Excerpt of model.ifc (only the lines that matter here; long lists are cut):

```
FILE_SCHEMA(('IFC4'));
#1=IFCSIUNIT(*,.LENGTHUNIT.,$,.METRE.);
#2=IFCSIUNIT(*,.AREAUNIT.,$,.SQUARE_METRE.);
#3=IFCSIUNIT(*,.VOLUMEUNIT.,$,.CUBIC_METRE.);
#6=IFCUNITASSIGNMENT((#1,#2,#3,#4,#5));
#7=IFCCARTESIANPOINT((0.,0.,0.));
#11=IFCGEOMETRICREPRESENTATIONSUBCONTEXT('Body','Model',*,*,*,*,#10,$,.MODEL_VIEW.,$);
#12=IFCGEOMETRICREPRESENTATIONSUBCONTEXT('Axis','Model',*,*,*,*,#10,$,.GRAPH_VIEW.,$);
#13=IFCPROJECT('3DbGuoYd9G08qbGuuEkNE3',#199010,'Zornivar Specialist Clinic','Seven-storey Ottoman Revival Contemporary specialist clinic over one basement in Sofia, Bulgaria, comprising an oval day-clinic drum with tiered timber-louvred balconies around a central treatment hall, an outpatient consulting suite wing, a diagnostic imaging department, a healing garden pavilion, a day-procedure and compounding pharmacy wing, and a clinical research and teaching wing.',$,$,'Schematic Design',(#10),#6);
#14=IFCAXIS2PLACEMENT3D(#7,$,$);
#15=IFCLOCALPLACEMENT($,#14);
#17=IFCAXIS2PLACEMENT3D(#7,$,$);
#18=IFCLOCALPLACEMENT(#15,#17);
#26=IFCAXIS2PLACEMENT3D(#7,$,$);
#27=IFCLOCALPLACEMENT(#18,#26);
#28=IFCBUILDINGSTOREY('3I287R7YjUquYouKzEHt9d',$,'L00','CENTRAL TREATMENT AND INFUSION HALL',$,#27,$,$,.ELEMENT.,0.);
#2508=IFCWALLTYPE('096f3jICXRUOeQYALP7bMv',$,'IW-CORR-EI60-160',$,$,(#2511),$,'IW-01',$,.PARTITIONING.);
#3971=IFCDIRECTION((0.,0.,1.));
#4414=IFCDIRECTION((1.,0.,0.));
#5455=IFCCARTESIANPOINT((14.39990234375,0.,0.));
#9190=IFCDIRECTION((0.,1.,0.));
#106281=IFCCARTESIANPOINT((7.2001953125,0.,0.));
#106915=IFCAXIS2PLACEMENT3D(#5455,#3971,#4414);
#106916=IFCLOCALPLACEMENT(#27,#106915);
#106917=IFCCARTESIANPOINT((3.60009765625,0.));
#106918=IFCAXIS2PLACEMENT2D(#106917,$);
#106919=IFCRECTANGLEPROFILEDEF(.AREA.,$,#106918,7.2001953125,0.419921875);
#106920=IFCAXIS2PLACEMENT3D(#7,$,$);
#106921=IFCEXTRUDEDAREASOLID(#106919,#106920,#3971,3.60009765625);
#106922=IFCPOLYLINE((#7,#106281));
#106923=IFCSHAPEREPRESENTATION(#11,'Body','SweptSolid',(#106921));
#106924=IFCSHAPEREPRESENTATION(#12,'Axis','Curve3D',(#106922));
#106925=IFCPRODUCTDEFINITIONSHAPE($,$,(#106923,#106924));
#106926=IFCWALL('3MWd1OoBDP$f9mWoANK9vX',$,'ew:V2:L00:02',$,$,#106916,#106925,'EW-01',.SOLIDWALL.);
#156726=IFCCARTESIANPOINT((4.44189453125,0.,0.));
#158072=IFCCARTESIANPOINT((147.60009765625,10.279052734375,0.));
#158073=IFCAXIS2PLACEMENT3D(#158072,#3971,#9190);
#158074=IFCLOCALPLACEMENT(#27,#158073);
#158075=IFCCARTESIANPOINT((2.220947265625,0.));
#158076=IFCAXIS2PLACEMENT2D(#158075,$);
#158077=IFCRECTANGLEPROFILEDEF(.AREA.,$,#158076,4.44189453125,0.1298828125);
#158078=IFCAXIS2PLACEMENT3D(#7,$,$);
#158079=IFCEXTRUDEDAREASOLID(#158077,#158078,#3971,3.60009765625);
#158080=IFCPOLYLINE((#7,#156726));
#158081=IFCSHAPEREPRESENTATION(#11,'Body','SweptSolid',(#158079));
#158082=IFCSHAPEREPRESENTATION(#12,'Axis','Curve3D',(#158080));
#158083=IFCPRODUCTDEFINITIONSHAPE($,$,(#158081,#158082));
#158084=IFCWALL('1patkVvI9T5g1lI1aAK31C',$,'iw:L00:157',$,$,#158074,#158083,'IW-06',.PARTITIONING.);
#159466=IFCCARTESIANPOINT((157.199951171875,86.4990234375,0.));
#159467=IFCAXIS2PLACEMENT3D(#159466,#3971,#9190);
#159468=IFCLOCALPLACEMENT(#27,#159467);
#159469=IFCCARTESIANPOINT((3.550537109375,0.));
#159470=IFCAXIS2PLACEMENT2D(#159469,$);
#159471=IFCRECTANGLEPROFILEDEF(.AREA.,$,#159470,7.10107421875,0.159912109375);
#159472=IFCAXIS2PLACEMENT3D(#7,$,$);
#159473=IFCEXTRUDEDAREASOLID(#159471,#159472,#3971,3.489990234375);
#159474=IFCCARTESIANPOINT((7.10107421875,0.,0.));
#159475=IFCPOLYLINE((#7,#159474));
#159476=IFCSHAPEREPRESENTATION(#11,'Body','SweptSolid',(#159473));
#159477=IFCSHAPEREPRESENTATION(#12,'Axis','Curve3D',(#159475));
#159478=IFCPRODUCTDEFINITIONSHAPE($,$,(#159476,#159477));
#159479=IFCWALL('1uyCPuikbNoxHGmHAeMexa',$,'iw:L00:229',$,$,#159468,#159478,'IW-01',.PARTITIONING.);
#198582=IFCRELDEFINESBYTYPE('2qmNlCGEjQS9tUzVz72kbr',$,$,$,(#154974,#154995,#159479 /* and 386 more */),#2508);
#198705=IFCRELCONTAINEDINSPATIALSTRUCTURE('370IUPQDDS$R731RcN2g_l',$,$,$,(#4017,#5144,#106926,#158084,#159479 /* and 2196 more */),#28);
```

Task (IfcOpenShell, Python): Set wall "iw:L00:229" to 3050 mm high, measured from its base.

```python
import ifcopenshell
import ifcopenshell.geom
import ifcopenshell.util.representation
import ifcopenshell.util.shape

model = ifcopenshell.open("model.ifc")
settings = ifcopenshell.geom.settings()


def volume(element):
    """Net volume in cubic metres, openings subtracted."""
    shape = ifcopenshell.geom.create_shape(settings, element)
    return ifcopenshell.util.shape.get_volume(shape.geometry)


wall = model.by_guid("1uyCPuikbNoxHGmHAeMexa")
before = volume(wall)

body = ifcopenshell.util.representation.get_representation(wall, "Model", "Body")
solid = body.Items[0]
old_height = solid.Depth
solid.Depth = 3.05
after = volume(wall)

print(f"height {old_height:g} -> {solid.Depth:g}, volume {before:.3f} -> {after:.3f} m3")

model.write("model_rev.ifc")
```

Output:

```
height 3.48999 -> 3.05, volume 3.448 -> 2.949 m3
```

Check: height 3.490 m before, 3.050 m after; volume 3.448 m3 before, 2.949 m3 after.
